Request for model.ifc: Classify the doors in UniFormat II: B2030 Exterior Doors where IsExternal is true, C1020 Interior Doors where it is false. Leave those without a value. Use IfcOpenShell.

First a look at what the model holds.

```python
import ifcopenshell
import ifcopenshell.util.element

model = ifcopenshell.open("model.ifc")
print(model.schema)
print("classifications:", [c.Name for c in model.by_type("IfcClassification")])
values = [ifcopenshell.util.element.get_pset(e, "Pset_DoorCommon", "IsExternal") for e in model.by_type("IfcDoor")]
for value in (True, False, None):
    print("IsExternal", value, values.count(value))
```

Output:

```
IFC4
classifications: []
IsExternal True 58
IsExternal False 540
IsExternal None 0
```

```python
import ifcopenshell
import ifcopenshell.api.classification
import ifcopenshell.util.element

model = ifcopenshell.open("model.ifc")

system = ifcopenshell.api.classification.add_classification(model, classification="UniFormat II")

doors = model.by_type("IfcDoor")
external = {e: ifcopenshell.util.element.get_pset(e, "Pset_DoorCommon", "IsExternal") for e in doors}
for flag, code, name in ((True, "B2030", "Exterior Doors"), (False, "C1020", "Interior Doors")):
    products = [e for e in doors if external[e] is flag]
    ifcopenshell.api.classification.add_reference(
        model, products=products, classification=system, identification=code, name=name
    )
    print(code, len(products))

model.write("model_edited.ifc")
```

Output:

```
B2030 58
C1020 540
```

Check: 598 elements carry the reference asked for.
